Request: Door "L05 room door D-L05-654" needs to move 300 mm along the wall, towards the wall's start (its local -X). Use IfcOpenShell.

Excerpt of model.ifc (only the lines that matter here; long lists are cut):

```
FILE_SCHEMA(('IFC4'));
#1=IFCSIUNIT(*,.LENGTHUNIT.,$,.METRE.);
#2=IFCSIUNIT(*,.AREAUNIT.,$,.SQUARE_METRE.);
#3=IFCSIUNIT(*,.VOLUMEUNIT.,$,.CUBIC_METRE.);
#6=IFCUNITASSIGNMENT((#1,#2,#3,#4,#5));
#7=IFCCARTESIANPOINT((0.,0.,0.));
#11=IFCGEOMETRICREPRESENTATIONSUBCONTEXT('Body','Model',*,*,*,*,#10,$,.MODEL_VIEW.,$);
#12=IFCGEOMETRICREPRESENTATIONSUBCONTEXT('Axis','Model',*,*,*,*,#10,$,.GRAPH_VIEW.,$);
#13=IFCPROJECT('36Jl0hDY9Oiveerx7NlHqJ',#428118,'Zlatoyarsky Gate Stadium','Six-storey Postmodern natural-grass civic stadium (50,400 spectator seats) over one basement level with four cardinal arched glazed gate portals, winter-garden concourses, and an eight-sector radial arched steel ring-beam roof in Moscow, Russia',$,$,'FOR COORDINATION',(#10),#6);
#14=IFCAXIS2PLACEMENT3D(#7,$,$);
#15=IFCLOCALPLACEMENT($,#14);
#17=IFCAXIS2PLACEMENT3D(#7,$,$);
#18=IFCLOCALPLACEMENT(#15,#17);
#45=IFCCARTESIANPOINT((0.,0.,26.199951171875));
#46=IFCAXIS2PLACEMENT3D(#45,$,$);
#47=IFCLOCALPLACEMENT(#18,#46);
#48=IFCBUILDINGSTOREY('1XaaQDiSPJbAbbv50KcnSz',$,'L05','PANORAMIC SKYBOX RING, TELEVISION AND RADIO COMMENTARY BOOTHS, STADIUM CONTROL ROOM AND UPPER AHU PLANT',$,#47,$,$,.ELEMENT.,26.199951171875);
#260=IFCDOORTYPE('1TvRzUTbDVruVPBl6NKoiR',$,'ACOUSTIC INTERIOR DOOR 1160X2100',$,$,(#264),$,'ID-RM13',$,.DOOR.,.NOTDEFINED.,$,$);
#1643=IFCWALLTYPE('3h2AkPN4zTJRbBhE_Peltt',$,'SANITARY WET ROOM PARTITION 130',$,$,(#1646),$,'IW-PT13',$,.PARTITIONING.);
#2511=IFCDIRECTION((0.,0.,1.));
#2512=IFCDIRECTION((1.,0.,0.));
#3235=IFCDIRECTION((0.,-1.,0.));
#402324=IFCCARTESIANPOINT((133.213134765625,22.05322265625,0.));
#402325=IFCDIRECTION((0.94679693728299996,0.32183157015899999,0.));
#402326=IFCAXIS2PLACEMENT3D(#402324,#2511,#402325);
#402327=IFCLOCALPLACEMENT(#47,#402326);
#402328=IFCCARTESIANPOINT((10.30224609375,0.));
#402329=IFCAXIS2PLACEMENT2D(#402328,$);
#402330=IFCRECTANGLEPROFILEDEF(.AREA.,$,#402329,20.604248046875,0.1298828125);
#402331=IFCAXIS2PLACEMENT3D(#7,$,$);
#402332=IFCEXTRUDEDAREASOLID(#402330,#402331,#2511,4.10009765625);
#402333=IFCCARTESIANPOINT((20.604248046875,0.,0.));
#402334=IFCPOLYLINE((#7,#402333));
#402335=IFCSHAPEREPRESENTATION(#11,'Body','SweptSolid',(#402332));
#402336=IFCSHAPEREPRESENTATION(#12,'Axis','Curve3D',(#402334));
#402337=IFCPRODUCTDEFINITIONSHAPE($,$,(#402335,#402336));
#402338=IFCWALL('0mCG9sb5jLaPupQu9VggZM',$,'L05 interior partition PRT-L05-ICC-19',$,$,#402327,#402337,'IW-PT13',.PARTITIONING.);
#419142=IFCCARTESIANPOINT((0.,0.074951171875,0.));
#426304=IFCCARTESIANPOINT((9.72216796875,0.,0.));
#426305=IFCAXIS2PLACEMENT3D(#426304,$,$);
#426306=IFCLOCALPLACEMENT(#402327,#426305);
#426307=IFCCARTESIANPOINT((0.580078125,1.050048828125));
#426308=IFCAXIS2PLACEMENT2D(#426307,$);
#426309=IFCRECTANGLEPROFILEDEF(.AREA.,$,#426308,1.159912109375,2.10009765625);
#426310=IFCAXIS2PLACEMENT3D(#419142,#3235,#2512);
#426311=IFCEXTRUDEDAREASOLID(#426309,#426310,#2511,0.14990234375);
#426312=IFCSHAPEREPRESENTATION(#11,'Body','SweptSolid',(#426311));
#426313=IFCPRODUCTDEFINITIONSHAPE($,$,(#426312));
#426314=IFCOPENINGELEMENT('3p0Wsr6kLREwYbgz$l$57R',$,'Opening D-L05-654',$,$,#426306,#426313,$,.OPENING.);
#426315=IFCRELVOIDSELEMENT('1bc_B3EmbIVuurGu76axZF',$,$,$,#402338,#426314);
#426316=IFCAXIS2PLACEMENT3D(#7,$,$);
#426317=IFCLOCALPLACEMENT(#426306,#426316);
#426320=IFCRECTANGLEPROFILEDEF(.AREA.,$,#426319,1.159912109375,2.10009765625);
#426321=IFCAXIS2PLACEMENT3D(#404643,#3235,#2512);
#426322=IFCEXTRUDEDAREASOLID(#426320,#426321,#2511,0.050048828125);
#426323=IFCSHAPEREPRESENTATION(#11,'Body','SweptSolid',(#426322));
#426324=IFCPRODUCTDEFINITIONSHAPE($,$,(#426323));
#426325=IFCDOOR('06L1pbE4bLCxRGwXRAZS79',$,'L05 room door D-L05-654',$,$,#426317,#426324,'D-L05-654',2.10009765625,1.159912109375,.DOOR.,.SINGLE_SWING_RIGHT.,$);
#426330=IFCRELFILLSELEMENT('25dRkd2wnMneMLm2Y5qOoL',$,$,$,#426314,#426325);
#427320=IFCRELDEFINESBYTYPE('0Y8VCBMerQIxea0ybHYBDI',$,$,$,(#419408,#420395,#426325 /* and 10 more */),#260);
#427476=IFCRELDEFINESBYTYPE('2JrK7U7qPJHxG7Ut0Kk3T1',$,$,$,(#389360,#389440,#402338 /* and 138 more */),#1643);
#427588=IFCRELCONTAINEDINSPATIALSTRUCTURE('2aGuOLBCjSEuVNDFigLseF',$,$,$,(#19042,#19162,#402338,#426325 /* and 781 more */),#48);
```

```python
import ifcopenshell
import ifcopenshell.api.geometry
import ifcopenshell.util.placement

model = ifcopenshell.open("model.ifc")

door = model.by_guid("06L1pbE4bLCxRGwXRAZS79")
opening = door.FillsVoids[0].RelatingOpeningElement
wall = opening.VoidsElements[0].RelatingBuildingElement

wall_matrix = ifcopenshell.util.placement.get_local_placement(wall.ObjectPlacement)
shift = wall_matrix[:3, 0] * -0.3
before = ifcopenshell.util.placement.get_local_placement(door.ObjectPlacement)[:3, 3].copy()

# The door is placed relative to its opening, so it follows when the opening moves.
matrix = ifcopenshell.util.placement.get_local_placement(opening.ObjectPlacement)
matrix[:3, 3] += shift
ifcopenshell.api.geometry.edit_object_placement(
    model, product=opening, matrix=matrix, is_si=False, should_transform_children=True
)

after = ifcopenshell.util.placement.get_local_placement(door.ObjectPlacement)[:3, 3]
print("door moved by", (after - before).round(3) + 0.0)

model.write("model_edited.ifc")
```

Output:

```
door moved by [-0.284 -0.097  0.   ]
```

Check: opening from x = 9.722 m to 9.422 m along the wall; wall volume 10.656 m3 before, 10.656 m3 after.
